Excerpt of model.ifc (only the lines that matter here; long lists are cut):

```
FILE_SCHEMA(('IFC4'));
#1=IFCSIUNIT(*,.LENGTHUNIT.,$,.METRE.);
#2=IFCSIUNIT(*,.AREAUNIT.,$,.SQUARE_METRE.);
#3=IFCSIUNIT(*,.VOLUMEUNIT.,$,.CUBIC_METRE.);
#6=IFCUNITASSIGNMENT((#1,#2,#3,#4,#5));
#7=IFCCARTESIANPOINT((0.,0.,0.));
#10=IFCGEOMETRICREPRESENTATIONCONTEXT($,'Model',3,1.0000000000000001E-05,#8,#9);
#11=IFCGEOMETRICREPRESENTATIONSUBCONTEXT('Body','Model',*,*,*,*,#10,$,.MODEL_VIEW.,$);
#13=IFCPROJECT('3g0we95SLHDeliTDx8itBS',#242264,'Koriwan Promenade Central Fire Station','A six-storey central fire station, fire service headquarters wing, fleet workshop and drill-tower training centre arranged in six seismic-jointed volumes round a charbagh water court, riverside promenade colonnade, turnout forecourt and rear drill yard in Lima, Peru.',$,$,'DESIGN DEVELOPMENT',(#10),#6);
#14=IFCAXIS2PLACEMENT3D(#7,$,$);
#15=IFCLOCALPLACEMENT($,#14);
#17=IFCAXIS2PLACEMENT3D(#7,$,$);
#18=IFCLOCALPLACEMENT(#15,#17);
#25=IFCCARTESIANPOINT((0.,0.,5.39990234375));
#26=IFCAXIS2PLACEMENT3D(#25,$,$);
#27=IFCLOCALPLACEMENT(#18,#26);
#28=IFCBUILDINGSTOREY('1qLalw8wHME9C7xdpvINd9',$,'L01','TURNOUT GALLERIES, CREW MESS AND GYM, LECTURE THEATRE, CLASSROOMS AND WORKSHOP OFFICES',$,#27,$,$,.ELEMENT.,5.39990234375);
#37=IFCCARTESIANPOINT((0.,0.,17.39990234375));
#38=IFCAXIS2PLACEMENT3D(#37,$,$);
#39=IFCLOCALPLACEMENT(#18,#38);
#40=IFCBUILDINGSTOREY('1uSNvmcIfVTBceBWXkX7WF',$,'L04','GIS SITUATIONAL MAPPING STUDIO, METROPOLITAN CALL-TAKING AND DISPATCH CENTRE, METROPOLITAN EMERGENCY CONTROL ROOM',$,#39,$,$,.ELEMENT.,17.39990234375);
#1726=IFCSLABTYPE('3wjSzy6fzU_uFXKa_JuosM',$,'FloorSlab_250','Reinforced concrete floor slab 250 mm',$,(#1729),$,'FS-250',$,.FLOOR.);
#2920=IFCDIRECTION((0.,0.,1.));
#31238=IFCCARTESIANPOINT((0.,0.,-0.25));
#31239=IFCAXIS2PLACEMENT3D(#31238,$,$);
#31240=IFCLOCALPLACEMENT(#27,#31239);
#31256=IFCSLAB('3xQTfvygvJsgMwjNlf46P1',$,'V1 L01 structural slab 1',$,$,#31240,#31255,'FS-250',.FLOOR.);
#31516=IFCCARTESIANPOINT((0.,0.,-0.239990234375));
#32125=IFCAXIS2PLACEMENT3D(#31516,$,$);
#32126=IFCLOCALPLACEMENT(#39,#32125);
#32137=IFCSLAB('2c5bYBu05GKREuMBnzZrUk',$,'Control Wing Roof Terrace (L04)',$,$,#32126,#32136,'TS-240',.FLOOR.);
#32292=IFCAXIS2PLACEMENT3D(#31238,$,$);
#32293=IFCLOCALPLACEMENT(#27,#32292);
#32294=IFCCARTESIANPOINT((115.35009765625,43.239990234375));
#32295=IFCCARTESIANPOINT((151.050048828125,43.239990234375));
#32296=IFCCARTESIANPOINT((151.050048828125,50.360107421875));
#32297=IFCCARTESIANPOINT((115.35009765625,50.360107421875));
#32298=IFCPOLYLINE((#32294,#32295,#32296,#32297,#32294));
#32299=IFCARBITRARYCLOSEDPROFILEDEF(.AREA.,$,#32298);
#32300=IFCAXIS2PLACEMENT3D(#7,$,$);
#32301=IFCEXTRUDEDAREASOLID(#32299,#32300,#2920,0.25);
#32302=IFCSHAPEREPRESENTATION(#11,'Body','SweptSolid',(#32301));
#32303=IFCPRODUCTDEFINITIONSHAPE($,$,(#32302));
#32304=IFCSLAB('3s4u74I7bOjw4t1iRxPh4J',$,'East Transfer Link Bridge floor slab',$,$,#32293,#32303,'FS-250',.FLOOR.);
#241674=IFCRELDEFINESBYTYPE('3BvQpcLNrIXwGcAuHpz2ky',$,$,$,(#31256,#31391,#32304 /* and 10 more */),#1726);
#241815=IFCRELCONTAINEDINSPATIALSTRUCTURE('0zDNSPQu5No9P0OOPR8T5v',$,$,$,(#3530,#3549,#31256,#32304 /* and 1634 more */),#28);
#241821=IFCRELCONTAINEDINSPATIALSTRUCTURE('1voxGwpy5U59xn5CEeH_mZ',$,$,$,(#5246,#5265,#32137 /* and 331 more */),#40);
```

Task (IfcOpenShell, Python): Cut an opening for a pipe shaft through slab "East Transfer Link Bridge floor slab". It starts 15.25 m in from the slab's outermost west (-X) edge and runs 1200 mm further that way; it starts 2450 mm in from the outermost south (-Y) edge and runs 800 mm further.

```python
import numpy as np
import ifcopenshell
import ifcopenshell.api.feature
import ifcopenshell.api.geometry
import ifcopenshell.api.root
import ifcopenshell.geom
import ifcopenshell.util.placement
import ifcopenshell.util.representation
import ifcopenshell.util.shape
import ifcopenshell.util.unit

model = ifcopenshell.open("model.ifc")
unit_scale = ifcopenshell.util.unit.calculate_unit_scale(model)
settings = ifcopenshell.geom.settings()


def volume(element):
    """Net volume in cubic metres, openings subtracted."""
    shape = ifcopenshell.geom.create_shape(settings, element)
    return ifcopenshell.util.shape.get_volume(shape.geometry)


slab = model.by_guid("3s4u74I7bOjw4t1iRxPh4J")
before = volume(slab)

# Extent in the slab's own axes, in metres. The edges named are its -X and -Y sides.
slab_shape = ifcopenshell.geom.create_shape(settings, slab)
vertices = ifcopenshell.util.shape.get_vertices(slab_shape.geometry)
x_min, y_min, bottom = vertices.min(axis=0)
top = vertices[:, 2].max()

opening = ifcopenshell.api.root.create_entity(model, ifc_class="IfcOpeningElement", name="Pipe shaft opening", predefined_type="OPENING")
context = ifcopenshell.util.representation.get_context(model, "Model", "Body", "MODEL_VIEW")
width, depth = 1.2, 0.8
outline = [(0.0, 0.0), (width, 0.0), (width, depth), (0.0, depth), (0.0, 0.0)]
# Overshoot both faces by 50 mm so the cut is clean.
shape = ifcopenshell.api.geometry.add_slab_representation(
    model, context=context, depth=top - bottom + 0.1, polyline=outline
)
ifcopenshell.api.geometry.assign_representation(model, product=opening, representation=shape)

matrix = ifcopenshell.util.placement.get_local_placement(slab.ObjectPlacement)
matrix[:, 3] = matrix @ np.append(np.array([x_min + 15.25, y_min + 2.45, bottom - 0.05]) / unit_scale, 1.0)
ifcopenshell.api.geometry.edit_object_placement(model, product=opening, matrix=matrix, is_si=False)
ifcopenshell.api.feature.add_feature(model, feature=opening, element=slab)

after = volume(slab)

print(f"slab volume {before:.3f} -> {after:.3f} m3")

model.write("model_edited.ifc")
```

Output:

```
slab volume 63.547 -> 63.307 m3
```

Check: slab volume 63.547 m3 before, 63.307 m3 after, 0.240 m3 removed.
